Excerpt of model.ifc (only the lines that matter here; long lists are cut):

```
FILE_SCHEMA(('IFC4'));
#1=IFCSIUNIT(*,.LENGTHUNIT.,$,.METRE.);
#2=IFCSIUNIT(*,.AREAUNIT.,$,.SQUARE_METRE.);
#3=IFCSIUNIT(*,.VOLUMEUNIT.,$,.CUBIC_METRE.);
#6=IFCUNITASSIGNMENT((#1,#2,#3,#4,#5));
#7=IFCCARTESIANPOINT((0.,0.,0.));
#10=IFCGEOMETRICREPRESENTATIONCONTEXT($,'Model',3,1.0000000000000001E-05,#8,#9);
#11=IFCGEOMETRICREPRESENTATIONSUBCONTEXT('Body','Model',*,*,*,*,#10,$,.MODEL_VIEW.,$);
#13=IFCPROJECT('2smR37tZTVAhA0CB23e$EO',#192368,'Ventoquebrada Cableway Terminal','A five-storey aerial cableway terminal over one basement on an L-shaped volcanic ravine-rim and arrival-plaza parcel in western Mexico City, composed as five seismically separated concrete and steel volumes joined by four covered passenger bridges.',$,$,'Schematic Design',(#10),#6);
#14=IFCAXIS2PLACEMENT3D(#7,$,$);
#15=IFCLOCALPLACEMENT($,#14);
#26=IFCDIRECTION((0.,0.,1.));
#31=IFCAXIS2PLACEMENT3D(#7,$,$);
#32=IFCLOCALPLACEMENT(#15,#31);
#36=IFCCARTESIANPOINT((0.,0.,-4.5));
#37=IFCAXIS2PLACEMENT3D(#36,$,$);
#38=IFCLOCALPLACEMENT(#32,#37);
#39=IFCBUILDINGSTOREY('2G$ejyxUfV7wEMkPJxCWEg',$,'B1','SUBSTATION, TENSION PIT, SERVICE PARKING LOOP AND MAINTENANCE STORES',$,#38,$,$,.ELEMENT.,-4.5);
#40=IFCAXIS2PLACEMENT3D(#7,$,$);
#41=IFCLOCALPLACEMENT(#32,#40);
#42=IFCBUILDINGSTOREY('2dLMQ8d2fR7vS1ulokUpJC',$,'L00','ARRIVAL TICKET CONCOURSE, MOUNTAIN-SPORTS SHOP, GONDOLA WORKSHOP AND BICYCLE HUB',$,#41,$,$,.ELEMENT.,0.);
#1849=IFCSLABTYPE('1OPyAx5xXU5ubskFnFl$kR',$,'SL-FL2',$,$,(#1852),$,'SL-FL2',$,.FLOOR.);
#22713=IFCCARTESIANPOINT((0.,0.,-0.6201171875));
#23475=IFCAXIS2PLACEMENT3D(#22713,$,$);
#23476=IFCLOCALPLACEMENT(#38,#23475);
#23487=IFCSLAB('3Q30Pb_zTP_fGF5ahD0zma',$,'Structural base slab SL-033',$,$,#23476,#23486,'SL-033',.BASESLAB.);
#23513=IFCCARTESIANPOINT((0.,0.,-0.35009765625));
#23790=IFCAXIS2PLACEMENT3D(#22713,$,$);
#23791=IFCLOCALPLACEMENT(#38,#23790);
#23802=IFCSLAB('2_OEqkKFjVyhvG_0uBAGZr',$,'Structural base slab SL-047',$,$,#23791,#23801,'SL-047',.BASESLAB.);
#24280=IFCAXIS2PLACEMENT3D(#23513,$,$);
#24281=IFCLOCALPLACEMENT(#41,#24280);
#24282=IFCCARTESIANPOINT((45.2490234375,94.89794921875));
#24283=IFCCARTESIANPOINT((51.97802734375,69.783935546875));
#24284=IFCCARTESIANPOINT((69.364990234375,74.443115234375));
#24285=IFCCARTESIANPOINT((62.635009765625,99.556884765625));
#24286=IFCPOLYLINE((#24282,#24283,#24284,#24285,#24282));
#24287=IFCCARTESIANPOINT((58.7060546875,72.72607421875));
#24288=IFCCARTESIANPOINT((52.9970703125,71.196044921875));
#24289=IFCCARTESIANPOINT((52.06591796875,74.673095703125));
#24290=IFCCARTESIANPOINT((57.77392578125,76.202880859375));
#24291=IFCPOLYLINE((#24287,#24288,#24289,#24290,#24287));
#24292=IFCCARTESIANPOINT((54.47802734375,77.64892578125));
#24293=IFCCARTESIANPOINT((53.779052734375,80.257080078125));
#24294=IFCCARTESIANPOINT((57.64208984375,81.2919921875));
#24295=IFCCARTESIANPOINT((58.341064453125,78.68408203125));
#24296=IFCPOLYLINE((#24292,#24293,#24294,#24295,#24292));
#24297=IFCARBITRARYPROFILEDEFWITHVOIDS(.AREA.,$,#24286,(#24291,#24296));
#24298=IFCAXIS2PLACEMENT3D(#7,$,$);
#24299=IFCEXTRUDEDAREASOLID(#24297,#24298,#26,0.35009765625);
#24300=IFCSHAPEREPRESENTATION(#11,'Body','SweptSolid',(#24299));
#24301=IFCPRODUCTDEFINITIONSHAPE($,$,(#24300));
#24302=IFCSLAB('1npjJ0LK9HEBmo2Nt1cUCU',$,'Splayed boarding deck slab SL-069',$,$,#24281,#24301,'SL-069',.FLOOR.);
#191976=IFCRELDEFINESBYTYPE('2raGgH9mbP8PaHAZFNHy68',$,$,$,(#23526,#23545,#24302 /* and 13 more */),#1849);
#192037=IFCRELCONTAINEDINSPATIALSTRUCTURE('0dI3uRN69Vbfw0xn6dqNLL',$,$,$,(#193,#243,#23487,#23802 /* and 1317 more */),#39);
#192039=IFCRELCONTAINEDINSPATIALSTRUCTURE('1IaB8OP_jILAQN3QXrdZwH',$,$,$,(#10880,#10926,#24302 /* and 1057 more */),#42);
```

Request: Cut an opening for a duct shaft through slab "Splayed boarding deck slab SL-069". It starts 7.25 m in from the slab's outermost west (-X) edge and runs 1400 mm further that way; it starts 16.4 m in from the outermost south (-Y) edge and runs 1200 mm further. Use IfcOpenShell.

```python
import numpy as np
import ifcopenshell
import ifcopenshell.api.feature
import ifcopenshell.api.geometry
import ifcopenshell.api.root
import ifcopenshell.geom
import ifcopenshell.util.placement
import ifcopenshell.util.representation
import ifcopenshell.util.shape
import ifcopenshell.util.unit

model = ifcopenshell.open("model.ifc")
unit_scale = ifcopenshell.util.unit.calculate_unit_scale(model)
settings = ifcopenshell.geom.settings()


def volume(element):
    """Net volume in cubic metres, openings subtracted."""
    shape = ifcopenshell.geom.create_shape(settings, element)
    return ifcopenshell.util.shape.get_volume(shape.geometry)


slab = model.by_guid("1npjJ0LK9HEBmo2Nt1cUCU")
before = volume(slab)

# Extent in the slab's own axes, in metres. The edges named are its -X and -Y sides.
slab_shape = ifcopenshell.geom.create_shape(settings, slab)
vertices = ifcopenshell.util.shape.get_vertices(slab_shape.geometry)
x_min, y_min, bottom = vertices.min(axis=0)
top = vertices[:, 2].max()

opening = ifcopenshell.api.root.create_entity(model, ifc_class="IfcOpeningElement", name="Duct shaft opening", predefined_type="OPENING")
context = ifcopenshell.util.representation.get_context(model, "Model", "Body", "MODEL_VIEW")
width, depth = 1.4, 1.2
outline = [(0.0, 0.0), (width, 0.0), (width, depth), (0.0, depth), (0.0, 0.0)]
# Overshoot both faces by 50 mm so the cut is clean.
shape = ifcopenshell.api.geometry.add_slab_representation(
    model, context=context, depth=top - bottom + 0.1, polyline=outline
)
ifcopenshell.api.geometry.assign_representation(model, product=opening, representation=shape)

matrix = ifcopenshell.util.placement.get_local_placement(slab.ObjectPlacement)
matrix[:, 3] = matrix @ np.append(np.array([x_min + 7.25, y_min + 16.4, bottom - 0.05]) / unit_scale, 1.0)
ifcopenshell.api.geometry.edit_object_placement(model, product=opening, matrix=matrix, is_si=False)
ifcopenshell.api.feature.add_feature(model, feature=opening, element=slab)

after = volume(slab)

print(f"slab volume {before:.3f} -> {after:.3f} m3")

model.write("model-out.ifc")
```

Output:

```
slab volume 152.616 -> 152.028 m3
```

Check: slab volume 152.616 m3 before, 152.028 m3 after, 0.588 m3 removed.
